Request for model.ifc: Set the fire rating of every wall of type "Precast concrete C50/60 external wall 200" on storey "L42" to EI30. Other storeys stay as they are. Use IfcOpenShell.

First a look at what the model holds.

```python
import ifcopenshell
import ifcopenshell.util.element

model = ifcopenshell.open("model.ifc")
print(model.schema)
storey = next(s for s in model.by_type("IfcBuildingStorey") if s.Name == "L42")
walls = [e for e in ifcopenshell.util.element.get_decomposition(storey) if e.is_a("IfcWall")]
seen = {}
for e in walls:
    element_type = ifcopenshell.util.element.get_type(e)
    key = (element_type.Name if element_type != e and element_type else None, ifcopenshell.util.element.get_pset(e, "Pset_WallCommon", "FireRating"))
    seen[key] = seen.get(key, 0) + 1
for (name, value), count in sorted(seen.items(), key=str):
    print(count, "x", name, "|", value)
```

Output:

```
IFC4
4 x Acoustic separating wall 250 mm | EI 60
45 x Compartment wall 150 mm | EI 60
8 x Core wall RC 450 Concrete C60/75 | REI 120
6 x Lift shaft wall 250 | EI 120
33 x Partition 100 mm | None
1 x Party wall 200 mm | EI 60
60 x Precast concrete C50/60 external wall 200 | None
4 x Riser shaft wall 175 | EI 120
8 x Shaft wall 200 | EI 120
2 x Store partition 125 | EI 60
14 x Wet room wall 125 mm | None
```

```python
import ifcopenshell
import ifcopenshell.api.pset
import ifcopenshell.util.element

model = ifcopenshell.open("model.ifc")

storey = next(s for s in model.by_type("IfcBuildingStorey") if s.Name == "L42")
walls = [e for e in ifcopenshell.util.element.get_decomposition(storey) if e.is_a("IfcWall")]

count = 0
for e in walls:
    element_type = ifcopenshell.util.element.get_type(e)
    if element_type in (None, e) or element_type.Name != "Precast concrete C50/60 external wall 200":
        continue
    found = ifcopenshell.util.element.get_pset(e, "Pset_WallCommon", should_inherit=False)
    if found:
        pset = model.by_id(found["id"])
        if len(ifcopenshell.util.element.get_elements_by_pset(pset)) > 1:
            pset = ifcopenshell.api.pset.unshare_pset(model, products=[e], pset=pset)[0]
    else:
        pset = ifcopenshell.api.pset.add_pset(model, product=e, name="Pset_WallCommon")
    ifcopenshell.api.pset.edit_pset(model, pset=pset, properties={"FireRating": "EI30"})
    count += 1

print(count, "walls updated")

model.write("model_edited.ifc")
```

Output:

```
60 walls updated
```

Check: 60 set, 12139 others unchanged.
